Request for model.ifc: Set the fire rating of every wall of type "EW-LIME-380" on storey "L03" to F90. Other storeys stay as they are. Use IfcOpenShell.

First a look at what the model holds.

```python
import ifcopenshell
import ifcopenshell.util.element

model = ifcopenshell.open("model.ifc")
print(model.schema)
storey = next(s for s in model.by_type("IfcBuildingStorey") if s.Name == "L03")
walls = [e for e in ifcopenshell.util.element.get_decomposition(storey) if e.is_a("IfcWall")]
seen = {}
for e in walls:
    element_type = ifcopenshell.util.element.get_type(e)
    key = (element_type.Name if element_type != e and element_type else None, ifcopenshell.util.element.get_pset(e, "Pset_WallCommon", "FireRating"))
    seen[key] = seen.get(key, 0) + 1
for (name, value), count in sorted(seen.items(), key=str):
    print(count, "x", name, "|", value)
```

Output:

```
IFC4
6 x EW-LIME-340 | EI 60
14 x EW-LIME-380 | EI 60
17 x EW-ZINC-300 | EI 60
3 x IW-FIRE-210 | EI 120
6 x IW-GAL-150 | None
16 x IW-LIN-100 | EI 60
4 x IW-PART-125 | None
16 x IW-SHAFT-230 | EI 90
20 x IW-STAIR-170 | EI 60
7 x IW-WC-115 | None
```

```python
import ifcopenshell
import ifcopenshell.api.pset
import ifcopenshell.util.element

model = ifcopenshell.open("model.ifc")

storey = next(s for s in model.by_type("IfcBuildingStorey") if s.Name == "L03")
walls = [e for e in ifcopenshell.util.element.get_decomposition(storey) if e.is_a("IfcWall")]

count = 0
for e in walls:
    element_type = ifcopenshell.util.element.get_type(e)
    if element_type in (None, e) or element_type.Name != "EW-LIME-380":
        continue
    # add_pset returns the element's existing set when there is one.
    pset = ifcopenshell.api.pset.add_pset(model, product=e, name="Pset_WallCommon")
    ifcopenshell.api.pset.edit_pset(model, pset=pset, properties={"FireRating": "F90"})
    count += 1

print(count, "walls updated")

model.write("model_updated.ifc")
```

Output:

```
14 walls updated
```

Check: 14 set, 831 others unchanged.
